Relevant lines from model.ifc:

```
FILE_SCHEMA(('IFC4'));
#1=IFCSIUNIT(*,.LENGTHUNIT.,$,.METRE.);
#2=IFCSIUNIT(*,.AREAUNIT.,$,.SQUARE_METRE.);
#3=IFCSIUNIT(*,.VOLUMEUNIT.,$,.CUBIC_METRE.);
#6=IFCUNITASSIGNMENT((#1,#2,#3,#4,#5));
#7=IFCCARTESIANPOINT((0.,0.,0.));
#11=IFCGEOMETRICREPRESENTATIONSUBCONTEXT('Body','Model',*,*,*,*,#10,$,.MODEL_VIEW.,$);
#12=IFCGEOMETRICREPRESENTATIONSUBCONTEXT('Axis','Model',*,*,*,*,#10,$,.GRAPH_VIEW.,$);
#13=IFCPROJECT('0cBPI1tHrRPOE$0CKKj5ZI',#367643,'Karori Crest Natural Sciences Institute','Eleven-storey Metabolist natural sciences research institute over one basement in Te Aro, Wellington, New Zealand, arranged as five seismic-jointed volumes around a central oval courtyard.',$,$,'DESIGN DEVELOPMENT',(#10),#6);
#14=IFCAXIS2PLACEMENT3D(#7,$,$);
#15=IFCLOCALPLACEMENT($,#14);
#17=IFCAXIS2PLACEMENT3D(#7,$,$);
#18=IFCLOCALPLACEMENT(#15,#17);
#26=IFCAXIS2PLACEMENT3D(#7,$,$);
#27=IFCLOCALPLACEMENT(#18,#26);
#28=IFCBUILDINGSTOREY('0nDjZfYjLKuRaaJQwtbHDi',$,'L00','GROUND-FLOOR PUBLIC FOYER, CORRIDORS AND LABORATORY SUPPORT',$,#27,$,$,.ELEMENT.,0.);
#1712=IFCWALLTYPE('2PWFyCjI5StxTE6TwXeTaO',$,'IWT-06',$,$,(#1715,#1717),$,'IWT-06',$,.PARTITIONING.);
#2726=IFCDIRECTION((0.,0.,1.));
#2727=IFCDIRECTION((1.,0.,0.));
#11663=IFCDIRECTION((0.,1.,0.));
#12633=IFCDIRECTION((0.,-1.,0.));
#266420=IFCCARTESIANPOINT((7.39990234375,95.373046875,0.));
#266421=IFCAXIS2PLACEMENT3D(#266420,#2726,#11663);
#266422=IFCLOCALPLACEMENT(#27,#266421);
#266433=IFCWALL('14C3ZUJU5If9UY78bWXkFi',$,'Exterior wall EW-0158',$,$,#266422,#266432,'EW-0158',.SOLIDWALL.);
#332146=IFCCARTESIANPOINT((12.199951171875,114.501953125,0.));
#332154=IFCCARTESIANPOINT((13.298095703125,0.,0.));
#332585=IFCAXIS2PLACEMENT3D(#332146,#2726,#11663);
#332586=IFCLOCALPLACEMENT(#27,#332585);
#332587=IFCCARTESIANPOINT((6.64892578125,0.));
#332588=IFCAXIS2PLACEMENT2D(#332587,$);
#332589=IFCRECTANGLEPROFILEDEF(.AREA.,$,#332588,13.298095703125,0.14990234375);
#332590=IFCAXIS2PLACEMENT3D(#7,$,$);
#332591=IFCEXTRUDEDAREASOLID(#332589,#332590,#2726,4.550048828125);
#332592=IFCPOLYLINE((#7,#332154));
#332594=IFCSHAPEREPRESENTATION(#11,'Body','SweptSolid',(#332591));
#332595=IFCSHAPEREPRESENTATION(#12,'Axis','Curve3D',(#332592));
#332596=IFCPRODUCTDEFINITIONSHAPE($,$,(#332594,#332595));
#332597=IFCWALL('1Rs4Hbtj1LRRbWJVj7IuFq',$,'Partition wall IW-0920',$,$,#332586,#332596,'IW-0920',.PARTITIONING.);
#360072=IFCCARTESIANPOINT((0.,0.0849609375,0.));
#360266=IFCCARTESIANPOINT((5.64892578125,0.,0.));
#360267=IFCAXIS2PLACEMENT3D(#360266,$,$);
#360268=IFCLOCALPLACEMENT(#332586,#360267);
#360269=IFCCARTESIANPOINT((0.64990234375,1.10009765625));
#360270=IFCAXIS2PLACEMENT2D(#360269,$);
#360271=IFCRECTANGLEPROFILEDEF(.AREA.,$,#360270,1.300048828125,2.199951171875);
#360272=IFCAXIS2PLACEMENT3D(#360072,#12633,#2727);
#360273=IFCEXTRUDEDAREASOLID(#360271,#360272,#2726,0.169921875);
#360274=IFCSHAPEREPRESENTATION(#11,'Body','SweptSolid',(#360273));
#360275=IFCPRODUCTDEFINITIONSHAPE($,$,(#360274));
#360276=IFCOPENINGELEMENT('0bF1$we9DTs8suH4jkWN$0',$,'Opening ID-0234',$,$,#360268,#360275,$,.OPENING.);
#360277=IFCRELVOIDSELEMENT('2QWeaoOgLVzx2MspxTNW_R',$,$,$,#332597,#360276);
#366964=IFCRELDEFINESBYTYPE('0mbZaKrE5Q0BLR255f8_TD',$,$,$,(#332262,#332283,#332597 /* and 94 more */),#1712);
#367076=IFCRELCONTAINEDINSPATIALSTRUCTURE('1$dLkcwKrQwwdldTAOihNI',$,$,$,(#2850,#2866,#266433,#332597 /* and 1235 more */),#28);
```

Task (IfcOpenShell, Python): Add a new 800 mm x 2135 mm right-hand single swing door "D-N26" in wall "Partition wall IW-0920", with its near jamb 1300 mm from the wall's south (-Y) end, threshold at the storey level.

```python
import numpy as np
import ifcopenshell
import ifcopenshell.api.feature
import ifcopenshell.api.geometry
import ifcopenshell.api.root
import ifcopenshell.api.spatial
import ifcopenshell.geom
import ifcopenshell.util.element
import ifcopenshell.util.placement
import ifcopenshell.util.representation
import ifcopenshell.util.shape
import ifcopenshell.util.unit

model = ifcopenshell.open("model.ifc")
unit_scale = ifcopenshell.util.unit.calculate_unit_scale(model)
settings = ifcopenshell.geom.settings()


def volume(element):
    """Net volume in cubic metres, openings subtracted."""
    shape = ifcopenshell.geom.create_shape(settings, element)
    return ifcopenshell.util.shape.get_volume(shape.geometry)


wall = model.by_guid("1Rs4Hbtj1LRRbWJVj7IuFq")
storey = ifcopenshell.util.element.get_container(wall, ifc_class="IfcBuildingStorey")
context = ifcopenshell.util.representation.get_context(model, "Model", "Body", "MODEL_VIEW")
before = volume(wall)

width, height, from_end, sill = 0.8, 2.135, 1.3, 0.0  # metres

# The wall runs along its own X axis, and the end named is its -X end.
wall_shape = ifcopenshell.geom.create_shape(settings, wall)
x, y, z = ifcopenshell.util.shape.get_vertices(wall_shape.geometry).T
start = x.min() + from_end
face, thickness = float(y.min()), float(y.max() - y.min())
wall_matrix = ifcopenshell.util.placement.get_local_placement(wall.ObjectPlacement)
level = ifcopenshell.util.placement.get_local_placement(storey.ObjectPlacement)[2, 3]


def in_wall(x, y):
    """Placement at x, y metres in the wall's axes, at sill height."""
    matrix = wall_matrix.copy()
    matrix[:, 3] = wall_matrix @ np.array([x / unit_scale, y / unit_scale, 0.0, 1.0])
    matrix[2, 3] = level + sill / unit_scale
    return matrix


# Opening: a box that overshoots both wall faces by 50 mm.
opening = ifcopenshell.api.root.create_entity(model, ifc_class="IfcOpeningElement", predefined_type="OPENING")
box = ifcopenshell.api.geometry.add_wall_representation(
    model, context=context, length=width, height=height, thickness=thickness + 0.1
)
ifcopenshell.api.geometry.assign_representation(model, product=opening, representation=box)
ifcopenshell.api.geometry.edit_object_placement(model, product=opening, matrix=in_wall(start, face - 0.05), is_si=False)
ifcopenshell.api.feature.add_feature(model, feature=opening, element=wall)

door = ifcopenshell.api.root.create_entity(model, ifc_class="IfcDoor", name="D-N26", predefined_type="DOOR")
door.OverallWidth, door.OverallHeight = width / unit_scale, height / unit_scale
door.OperationType = "SINGLE_SWING_RIGHT"
body = ifcopenshell.api.geometry.add_door_representation(
    model,
    context=context,
    overall_width=door.OverallWidth,
    overall_height=door.OverallHeight,
    operation_type="SINGLE_SWING_RIGHT",
    lining_properties={"LiningDepth": thickness / unit_scale, "ThresholdDepth": thickness / unit_scale},
)
ifcopenshell.api.geometry.assign_representation(model, product=door, representation=body)
ifcopenshell.api.spatial.assign_container(model, products=[door], relating_structure=storey)
ifcopenshell.api.feature.add_filling(model, opening=opening, element=door)

# The lining spans the wall, so the door starts at the wall face.
ifcopenshell.api.geometry.edit_object_placement(model, product=door, matrix=in_wall(start, face), is_si=False)

after = volume(wall)

print(f"wall volume {before:.3f} -> {after:.3f} m3")

model.write("model_edited.ifc")
```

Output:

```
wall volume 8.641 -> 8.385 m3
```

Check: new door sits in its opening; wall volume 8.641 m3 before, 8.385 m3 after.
